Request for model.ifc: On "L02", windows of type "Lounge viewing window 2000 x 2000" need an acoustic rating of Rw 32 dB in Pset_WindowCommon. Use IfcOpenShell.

First a look at what the model holds.

```python
import ifcopenshell
import ifcopenshell.util.element

model = ifcopenshell.open("model.ifc")
print(model.schema)
storey = next(s for s in model.by_type("IfcBuildingStorey") if s.Name == "L02")
windows = [e for e in ifcopenshell.util.element.get_decomposition(storey) if e.is_a("IfcWindow")]
seen = {}
for e in windows:
    element_type = ifcopenshell.util.element.get_type(e)
    key = (element_type.Name if element_type != e and element_type else None, ifcopenshell.util.element.get_pset(e, "Pset_WindowCommon", "AcousticRating"))
    seen[key] = seen.get(key, 0) + 1
for (name, value), count in sorted(seen.items(), key=str):
    print(count, "x", name, "|", value)
```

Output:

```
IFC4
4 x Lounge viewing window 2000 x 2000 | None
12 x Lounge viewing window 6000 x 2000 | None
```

```python
import ifcopenshell
import ifcopenshell.api.pset
import ifcopenshell.util.element

model = ifcopenshell.open("model.ifc")

storey = next(s for s in model.by_type("IfcBuildingStorey") if s.Name == "L02")
windows = [e for e in ifcopenshell.util.element.get_decomposition(storey) if e.is_a("IfcWindow")]

count = 0
for e in windows:
    element_type = ifcopenshell.util.element.get_type(e)
    if element_type in (None, e) or element_type.Name != "Lounge viewing window 2000 x 2000":
        continue
    # add_pset returns the element's existing set when there is one.
    pset = ifcopenshell.api.pset.add_pset(model, product=e, name="Pset_WindowCommon")
    ifcopenshell.api.pset.edit_pset(model, pset=pset, properties={"AcousticRating": "Rw 32 dB"})
    count += 1

print(count, "windows updated")

model.write("model_rev.ifc")
```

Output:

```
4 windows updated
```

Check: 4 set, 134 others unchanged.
